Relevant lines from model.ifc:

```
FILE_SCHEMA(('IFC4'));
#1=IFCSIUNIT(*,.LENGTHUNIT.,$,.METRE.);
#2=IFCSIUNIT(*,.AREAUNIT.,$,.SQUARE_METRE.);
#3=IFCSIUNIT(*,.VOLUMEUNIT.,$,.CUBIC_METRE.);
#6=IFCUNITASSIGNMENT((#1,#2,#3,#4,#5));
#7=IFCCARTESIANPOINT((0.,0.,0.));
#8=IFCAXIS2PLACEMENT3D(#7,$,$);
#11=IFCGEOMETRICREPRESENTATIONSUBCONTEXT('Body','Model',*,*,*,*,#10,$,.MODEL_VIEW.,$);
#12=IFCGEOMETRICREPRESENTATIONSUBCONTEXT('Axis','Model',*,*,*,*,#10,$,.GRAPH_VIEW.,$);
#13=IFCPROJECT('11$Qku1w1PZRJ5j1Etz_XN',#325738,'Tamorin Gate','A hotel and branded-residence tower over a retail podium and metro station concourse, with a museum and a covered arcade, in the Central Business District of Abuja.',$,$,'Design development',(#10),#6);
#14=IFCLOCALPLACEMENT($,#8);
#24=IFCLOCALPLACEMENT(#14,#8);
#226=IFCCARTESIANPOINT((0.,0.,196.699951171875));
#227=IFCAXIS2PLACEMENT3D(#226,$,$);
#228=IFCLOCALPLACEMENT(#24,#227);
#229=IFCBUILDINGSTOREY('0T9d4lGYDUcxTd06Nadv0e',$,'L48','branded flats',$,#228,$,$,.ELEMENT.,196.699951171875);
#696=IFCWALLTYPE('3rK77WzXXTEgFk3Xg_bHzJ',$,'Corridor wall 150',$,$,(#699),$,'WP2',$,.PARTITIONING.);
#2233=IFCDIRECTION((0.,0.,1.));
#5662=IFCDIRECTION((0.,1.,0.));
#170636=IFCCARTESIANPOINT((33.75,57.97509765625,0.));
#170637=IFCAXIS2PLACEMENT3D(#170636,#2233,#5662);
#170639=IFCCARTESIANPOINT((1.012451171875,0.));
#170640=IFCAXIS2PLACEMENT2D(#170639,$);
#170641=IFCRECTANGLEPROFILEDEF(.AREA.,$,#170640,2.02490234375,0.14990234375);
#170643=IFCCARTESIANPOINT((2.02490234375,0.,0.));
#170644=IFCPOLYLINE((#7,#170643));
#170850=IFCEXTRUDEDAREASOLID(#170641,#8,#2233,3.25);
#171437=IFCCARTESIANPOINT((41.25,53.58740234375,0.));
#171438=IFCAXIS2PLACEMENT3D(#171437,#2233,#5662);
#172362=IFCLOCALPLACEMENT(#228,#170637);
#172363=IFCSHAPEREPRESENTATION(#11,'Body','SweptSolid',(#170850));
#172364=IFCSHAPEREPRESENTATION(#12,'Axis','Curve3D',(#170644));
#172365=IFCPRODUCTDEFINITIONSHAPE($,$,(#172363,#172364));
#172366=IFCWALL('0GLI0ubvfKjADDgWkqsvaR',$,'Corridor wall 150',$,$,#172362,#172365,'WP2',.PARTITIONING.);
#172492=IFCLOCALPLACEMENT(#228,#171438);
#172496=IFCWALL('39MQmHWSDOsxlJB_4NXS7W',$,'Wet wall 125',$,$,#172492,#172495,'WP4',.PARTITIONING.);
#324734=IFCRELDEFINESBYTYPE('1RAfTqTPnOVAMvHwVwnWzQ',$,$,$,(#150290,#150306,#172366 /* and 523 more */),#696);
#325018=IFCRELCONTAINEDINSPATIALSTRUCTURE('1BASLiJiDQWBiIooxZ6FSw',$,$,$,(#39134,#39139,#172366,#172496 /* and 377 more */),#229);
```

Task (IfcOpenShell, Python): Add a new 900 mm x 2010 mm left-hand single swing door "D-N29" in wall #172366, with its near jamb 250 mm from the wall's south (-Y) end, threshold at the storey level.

```python
import numpy as np
import ifcopenshell
import ifcopenshell.api.feature
import ifcopenshell.api.geometry
import ifcopenshell.api.root
import ifcopenshell.api.spatial
import ifcopenshell.geom
import ifcopenshell.util.element
import ifcopenshell.util.placement
import ifcopenshell.util.representation
import ifcopenshell.util.shape
import ifcopenshell.util.unit

model = ifcopenshell.open("model.ifc")
unit_scale = ifcopenshell.util.unit.calculate_unit_scale(model)
settings = ifcopenshell.geom.settings()


def volume(element):
    """Net volume in cubic metres, openings subtracted."""
    shape = ifcopenshell.geom.create_shape(settings, element)
    return ifcopenshell.util.shape.get_volume(shape.geometry)


wall = model.by_guid("0GLI0ubvfKjADDgWkqsvaR")
storey = ifcopenshell.util.element.get_container(wall, ifc_class="IfcBuildingStorey")
context = ifcopenshell.util.representation.get_context(model, "Model", "Body", "MODEL_VIEW")
before = volume(wall)

width, height, from_end, sill = 0.9, 2.01, 0.25, 0.0  # metres

# The wall runs along its own X axis, and the end named is its -X end.
wall_shape = ifcopenshell.geom.create_shape(settings, wall)
x, y, z = ifcopenshell.util.shape.get_vertices(wall_shape.geometry).T
start = x.min() + from_end
face, thickness = float(y.min()), float(y.max() - y.min())
wall_matrix = ifcopenshell.util.placement.get_local_placement(wall.ObjectPlacement)
level = ifcopenshell.util.placement.get_local_placement(storey.ObjectPlacement)[2, 3]


def in_wall(x, y):
    """Placement at x, y metres in the wall's axes, at sill height."""
    matrix = wall_matrix.copy()
    matrix[:, 3] = wall_matrix @ np.array([x / unit_scale, y / unit_scale, 0.0, 1.0])
    matrix[2, 3] = level + sill / unit_scale
    return matrix


# Opening: a box that overshoots both wall faces by 50 mm.
opening = ifcopenshell.api.root.create_entity(model, ifc_class="IfcOpeningElement", predefined_type="OPENING")
box = ifcopenshell.api.geometry.add_wall_representation(
    model, context=context, length=width, height=height, thickness=thickness + 0.1
)
ifcopenshell.api.geometry.assign_representation(model, product=opening, representation=box)
ifcopenshell.api.geometry.edit_object_placement(model, product=opening, matrix=in_wall(start, face - 0.05), is_si=False)
ifcopenshell.api.feature.add_feature(model, feature=opening, element=wall)

door = ifcopenshell.api.root.create_entity(model, ifc_class="IfcDoor", name="D-N29", predefined_type="DOOR")
door.OverallWidth, door.OverallHeight = width / unit_scale, height / unit_scale
door.OperationType = "SINGLE_SWING_LEFT"
body = ifcopenshell.api.geometry.add_door_representation(
    model,
    context=context,
    overall_width=door.OverallWidth,
    overall_height=door.OverallHeight,
    operation_type="SINGLE_SWING_LEFT",
    lining_properties={"LiningDepth": thickness / unit_scale, "ThresholdDepth": thickness / unit_scale},
)
ifcopenshell.api.geometry.assign_representation(model, product=door, representation=body)
ifcopenshell.api.spatial.assign_container(model, products=[door], relating_structure=storey)
ifcopenshell.api.feature.add_filling(model, opening=opening, element=door)

# The lining spans the wall, so the door starts at the wall face.
ifcopenshell.api.geometry.edit_object_placement(model, product=door, matrix=in_wall(start, face), is_si=False)

after = volume(wall)

print(f"wall volume {before:.3f} -> {after:.3f} m3")

model.write("model_v2.ifc")
```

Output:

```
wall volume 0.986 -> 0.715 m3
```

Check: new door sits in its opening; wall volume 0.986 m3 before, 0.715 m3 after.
